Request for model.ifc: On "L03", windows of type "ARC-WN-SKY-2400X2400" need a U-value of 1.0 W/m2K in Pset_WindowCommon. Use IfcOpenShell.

First a look at what the model holds.

```python
import ifcopenshell
import ifcopenshell.util.element

model = ifcopenshell.open("model.ifc")
print(model.schema)
storey = next(s for s in model.by_type("IfcBuildingStorey") if s.Name == "L03")
windows = [e for e in ifcopenshell.util.element.get_decomposition(storey) if e.is_a("IfcWindow")]
seen = {}
for e in windows:
    element_type = ifcopenshell.util.element.get_type(e)
    key = (element_type.Name if element_type != e and element_type else None, ifcopenshell.util.element.get_pset(e, "Pset_WindowCommon", "ThermalTransmittance"))
    seen[key] = seen.get(key, 0) + 1
for (name, value), count in sorted(seen.items(), key=str):
    print(count, "x", name, "|", value)
```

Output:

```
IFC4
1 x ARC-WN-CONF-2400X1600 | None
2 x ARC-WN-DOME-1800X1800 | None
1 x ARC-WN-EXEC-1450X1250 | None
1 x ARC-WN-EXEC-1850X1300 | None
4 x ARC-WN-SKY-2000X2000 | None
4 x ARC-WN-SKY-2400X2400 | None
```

```python
import ifcopenshell
import ifcopenshell.api.pset
import ifcopenshell.util.element

model = ifcopenshell.open("model.ifc")

storey = next(s for s in model.by_type("IfcBuildingStorey") if s.Name == "L03")
windows = [e for e in ifcopenshell.util.element.get_decomposition(storey) if e.is_a("IfcWindow")]

count = 0
for e in windows:
    element_type = ifcopenshell.util.element.get_type(e)
    if element_type in (None, e) or element_type.Name != "ARC-WN-SKY-2400X2400":
        continue
    # add_pset returns the element's existing set when there is one.
    pset = ifcopenshell.api.pset.add_pset(model, product=e, name="Pset_WindowCommon")
    ifcopenshell.api.pset.edit_pset(model, pset=pset, properties={"ThermalTransmittance": 1.0})
    count += 1

print(count, "windows updated")

model.write("model_edited.ifc")
```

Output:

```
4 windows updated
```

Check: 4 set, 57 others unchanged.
